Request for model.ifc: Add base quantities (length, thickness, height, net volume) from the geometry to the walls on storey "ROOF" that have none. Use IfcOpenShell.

First a look at what the model holds.

```python
import ifcopenshell
import ifcopenshell.util.element
import ifcopenshell.util.unit

model = ifcopenshell.open("model.ifc")
print(model.schema)
for unit_type in ("LENGTHUNIT", "AREAUNIT", "VOLUMEUNIT"):
    print(unit_type, ifcopenshell.util.unit.calculate_unit_scale(model, unit_type))
storey = next(s for s in model.by_type("IfcBuildingStorey") if s.Name == "ROOF")
walls = [e for e in ifcopenshell.util.element.get_decomposition(storey) if e.is_a("IfcWall")]
for e in sorted(walls, key=lambda e: e.id()):
    print(e.id(), e.is_a(), e.Name, list(ifcopenshell.util.element.get_psets(e, qtos_only=True)), sep=" | ")
```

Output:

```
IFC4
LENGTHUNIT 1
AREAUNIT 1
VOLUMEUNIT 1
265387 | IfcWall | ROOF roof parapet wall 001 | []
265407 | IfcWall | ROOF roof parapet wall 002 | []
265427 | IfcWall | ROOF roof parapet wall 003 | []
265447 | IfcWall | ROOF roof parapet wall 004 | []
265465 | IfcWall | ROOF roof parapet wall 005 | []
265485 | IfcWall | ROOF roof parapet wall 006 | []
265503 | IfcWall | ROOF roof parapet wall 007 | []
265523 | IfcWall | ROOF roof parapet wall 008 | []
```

```python
import ifcopenshell
import ifcopenshell.api.pset
import ifcopenshell.geom
import ifcopenshell.util.element
import ifcopenshell.util.shape
import ifcopenshell.util.unit

model = ifcopenshell.open("model.ifc")
unit_scale = ifcopenshell.util.unit.calculate_unit_scale(model)
volume_scale = ifcopenshell.util.unit.calculate_unit_scale(model, "VOLUMEUNIT")
settings = ifcopenshell.geom.settings()

storey = next(s for s in model.by_type("IfcBuildingStorey") if s.Name == "ROOF")
walls = [e for e in ifcopenshell.util.element.get_decomposition(storey) if e.is_a("IfcWall")]

for e in sorted(walls, key=lambda e: e.id()):
    if ifcopenshell.util.element.get_psets(e, qtos_only=True, should_inherit=False):
        continue
    # Geometry comes back in metres, in the element's own axes.
    shape = ifcopenshell.geom.create_shape(settings, e)
    values = {
        "Length": ifcopenshell.util.shape.get_x(shape.geometry) / unit_scale,
        "Width": ifcopenshell.util.shape.get_y(shape.geometry) / unit_scale,
        "Height": ifcopenshell.util.shape.get_z(shape.geometry) / unit_scale,
        "NetVolume": ifcopenshell.util.shape.get_volume(shape.geometry) / volume_scale,
    }
    qto = ifcopenshell.api.pset.add_qto(model, product=e, name="Qto_WallBaseQuantities")
    ifcopenshell.api.pset.edit_qto(model, qto=qto, properties=values)
    print(e.id(), {k: round(v, 3) for k, v in values.items()})

model.write("model-out.ifc")
```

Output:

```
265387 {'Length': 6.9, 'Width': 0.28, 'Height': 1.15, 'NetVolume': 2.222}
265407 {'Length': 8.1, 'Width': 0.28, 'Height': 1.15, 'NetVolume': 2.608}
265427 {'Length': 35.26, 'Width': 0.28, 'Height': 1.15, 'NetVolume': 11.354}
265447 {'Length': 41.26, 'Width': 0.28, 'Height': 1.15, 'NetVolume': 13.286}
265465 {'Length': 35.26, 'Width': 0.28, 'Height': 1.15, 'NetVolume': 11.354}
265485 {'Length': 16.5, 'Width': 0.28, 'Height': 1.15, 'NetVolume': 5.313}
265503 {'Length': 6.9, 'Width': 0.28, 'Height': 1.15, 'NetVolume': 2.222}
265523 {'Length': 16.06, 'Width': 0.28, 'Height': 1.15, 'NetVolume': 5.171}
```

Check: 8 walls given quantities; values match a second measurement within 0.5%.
